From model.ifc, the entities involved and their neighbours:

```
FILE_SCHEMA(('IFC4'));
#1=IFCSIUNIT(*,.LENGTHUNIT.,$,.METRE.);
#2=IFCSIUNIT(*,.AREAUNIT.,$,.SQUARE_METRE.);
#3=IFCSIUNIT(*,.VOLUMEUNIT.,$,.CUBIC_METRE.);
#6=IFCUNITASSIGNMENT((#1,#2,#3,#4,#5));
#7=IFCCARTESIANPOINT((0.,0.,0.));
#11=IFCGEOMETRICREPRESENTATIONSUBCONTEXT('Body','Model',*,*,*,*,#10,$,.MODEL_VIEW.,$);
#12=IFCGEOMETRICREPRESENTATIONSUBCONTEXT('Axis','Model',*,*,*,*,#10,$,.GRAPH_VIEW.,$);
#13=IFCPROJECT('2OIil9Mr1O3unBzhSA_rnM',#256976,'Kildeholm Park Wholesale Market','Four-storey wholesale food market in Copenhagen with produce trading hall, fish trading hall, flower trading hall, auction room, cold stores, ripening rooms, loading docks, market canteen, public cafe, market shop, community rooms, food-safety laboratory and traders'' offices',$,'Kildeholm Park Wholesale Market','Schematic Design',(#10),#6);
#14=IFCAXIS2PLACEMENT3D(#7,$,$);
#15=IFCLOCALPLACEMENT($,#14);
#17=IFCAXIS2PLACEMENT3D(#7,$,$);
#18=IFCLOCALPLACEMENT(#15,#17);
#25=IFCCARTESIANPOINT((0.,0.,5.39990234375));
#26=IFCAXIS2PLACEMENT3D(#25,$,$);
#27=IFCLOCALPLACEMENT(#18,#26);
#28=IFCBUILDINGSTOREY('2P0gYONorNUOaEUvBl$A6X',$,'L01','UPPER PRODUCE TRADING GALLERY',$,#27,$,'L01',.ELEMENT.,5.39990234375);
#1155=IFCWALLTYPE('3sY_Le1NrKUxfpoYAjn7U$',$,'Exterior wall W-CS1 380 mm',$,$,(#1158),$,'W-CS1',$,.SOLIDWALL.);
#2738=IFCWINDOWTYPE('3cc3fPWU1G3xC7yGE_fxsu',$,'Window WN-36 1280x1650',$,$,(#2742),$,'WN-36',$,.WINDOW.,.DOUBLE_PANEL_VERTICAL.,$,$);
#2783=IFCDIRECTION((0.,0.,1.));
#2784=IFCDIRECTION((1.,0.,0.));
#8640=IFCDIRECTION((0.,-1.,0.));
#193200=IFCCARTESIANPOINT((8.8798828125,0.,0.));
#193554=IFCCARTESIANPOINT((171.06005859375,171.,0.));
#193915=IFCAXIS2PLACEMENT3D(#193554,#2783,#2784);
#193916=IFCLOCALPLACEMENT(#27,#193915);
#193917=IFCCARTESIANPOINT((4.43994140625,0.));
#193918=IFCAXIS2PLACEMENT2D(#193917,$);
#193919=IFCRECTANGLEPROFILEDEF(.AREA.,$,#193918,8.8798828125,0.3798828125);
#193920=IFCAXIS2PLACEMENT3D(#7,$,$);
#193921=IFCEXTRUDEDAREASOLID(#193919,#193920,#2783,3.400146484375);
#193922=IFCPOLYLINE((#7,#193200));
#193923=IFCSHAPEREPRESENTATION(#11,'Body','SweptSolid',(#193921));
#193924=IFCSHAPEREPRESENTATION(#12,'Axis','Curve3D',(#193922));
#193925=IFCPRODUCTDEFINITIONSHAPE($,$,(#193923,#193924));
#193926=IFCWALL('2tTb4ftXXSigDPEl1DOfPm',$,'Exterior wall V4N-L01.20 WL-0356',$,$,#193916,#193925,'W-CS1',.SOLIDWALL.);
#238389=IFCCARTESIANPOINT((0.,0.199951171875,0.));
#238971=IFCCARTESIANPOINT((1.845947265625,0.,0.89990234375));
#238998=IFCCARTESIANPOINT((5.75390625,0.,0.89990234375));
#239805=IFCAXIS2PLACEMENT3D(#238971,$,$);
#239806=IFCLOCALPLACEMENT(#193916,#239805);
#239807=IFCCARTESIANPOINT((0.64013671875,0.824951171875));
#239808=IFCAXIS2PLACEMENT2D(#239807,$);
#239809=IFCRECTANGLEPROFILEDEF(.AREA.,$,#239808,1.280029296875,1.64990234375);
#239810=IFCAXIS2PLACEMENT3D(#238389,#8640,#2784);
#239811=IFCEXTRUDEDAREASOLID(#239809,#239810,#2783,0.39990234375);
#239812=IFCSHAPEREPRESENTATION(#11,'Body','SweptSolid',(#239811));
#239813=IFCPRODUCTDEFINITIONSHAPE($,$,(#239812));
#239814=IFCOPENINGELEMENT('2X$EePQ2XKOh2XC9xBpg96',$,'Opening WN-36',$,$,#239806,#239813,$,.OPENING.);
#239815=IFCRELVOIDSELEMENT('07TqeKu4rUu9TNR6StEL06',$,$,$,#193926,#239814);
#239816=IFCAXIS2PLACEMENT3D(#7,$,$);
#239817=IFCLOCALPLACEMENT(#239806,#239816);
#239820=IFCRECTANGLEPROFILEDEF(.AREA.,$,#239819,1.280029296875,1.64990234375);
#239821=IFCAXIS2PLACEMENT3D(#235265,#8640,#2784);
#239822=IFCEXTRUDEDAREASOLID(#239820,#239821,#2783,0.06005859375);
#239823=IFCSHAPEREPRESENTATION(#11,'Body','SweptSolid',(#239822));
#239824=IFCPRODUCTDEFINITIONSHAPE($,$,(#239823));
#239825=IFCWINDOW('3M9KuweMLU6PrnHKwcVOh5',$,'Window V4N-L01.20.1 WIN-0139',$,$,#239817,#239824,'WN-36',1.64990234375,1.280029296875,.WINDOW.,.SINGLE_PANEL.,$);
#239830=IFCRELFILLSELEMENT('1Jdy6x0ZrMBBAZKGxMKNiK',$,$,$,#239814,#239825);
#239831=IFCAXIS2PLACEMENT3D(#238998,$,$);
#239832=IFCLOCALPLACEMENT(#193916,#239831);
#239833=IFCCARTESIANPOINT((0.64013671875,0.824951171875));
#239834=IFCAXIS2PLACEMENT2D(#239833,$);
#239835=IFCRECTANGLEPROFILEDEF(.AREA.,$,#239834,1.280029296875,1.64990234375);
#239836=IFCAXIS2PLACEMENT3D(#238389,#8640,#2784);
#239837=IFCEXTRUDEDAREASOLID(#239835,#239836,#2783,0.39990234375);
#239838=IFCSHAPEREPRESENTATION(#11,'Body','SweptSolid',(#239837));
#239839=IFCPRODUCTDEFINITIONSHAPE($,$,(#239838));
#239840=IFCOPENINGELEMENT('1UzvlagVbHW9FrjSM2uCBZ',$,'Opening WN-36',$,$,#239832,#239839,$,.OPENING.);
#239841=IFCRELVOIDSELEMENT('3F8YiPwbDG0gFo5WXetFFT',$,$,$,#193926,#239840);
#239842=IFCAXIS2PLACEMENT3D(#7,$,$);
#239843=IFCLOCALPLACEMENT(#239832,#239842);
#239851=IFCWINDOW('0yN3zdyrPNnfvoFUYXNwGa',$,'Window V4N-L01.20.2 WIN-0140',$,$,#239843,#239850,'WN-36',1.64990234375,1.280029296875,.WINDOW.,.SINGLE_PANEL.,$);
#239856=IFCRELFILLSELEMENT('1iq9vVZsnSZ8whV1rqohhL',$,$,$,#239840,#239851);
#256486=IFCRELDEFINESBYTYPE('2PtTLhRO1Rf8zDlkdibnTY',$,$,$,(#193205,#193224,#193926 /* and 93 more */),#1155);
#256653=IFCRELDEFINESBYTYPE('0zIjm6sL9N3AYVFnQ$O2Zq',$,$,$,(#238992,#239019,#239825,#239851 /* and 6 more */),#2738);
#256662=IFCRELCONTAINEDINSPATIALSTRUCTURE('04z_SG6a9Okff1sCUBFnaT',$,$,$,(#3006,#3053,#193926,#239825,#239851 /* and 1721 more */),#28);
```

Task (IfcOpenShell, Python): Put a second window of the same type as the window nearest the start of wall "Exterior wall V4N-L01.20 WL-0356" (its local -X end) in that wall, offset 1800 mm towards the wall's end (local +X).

```python
import ifcopenshell
import ifcopenshell.api.feature
import ifcopenshell.api.geometry
import ifcopenshell.api.root
import ifcopenshell.geom
import ifcopenshell.util.element
import ifcopenshell.util.placement
import ifcopenshell.util.shape
import ifcopenshell.util.unit

model = ifcopenshell.open("model.ifc")
unit_scale = ifcopenshell.util.unit.calculate_unit_scale(model)
settings = ifcopenshell.geom.settings()


def volume(element):
    """Net volume in cubic metres, openings subtracted."""
    shape = ifcopenshell.geom.create_shape(settings, element)
    return ifcopenshell.util.shape.get_volume(shape.geometry)


window = model.by_id(239825)
opening = window.FillsVoids[0].RelatingOpeningElement
wall = opening.VoidsElements[0].RelatingBuildingElement
before = volume(wall)
shift = ifcopenshell.util.placement.get_local_placement(wall.ObjectPlacement)[:3, 0] * 1.8 / unit_scale

# copy_class copies the void relationship, type, container and properties, but no geometry.
new_opening = ifcopenshell.api.root.copy_class(model, product=opening)
new_opening.Representation = ifcopenshell.util.element.copy_deep(
    model, opening.Representation, exclude=["IfcGeometricRepresentationContext", "IfcRepresentationMap"]
)
new_window = ifcopenshell.api.root.copy_class(model, product=window)
new_window.Representation = ifcopenshell.util.element.copy_deep(
    model, window.Representation, exclude=["IfcGeometricRepresentationContext", "IfcRepresentationMap"]
)
new_window.Tag = None
ifcopenshell.api.feature.add_filling(model, opening=new_opening, element=new_window)

for old, new in ((opening, new_opening), (window, new_window)):
    matrix = ifcopenshell.util.placement.get_local_placement(old.ObjectPlacement)
    matrix[:3, 3] += shift
    ifcopenshell.api.geometry.edit_object_placement(model, product=new, matrix=matrix, is_si=False)

after = volume(wall)

print(f"wall volume {before:.3f} -> {after:.3f} m3")

model.write("model_edited.ifc")
```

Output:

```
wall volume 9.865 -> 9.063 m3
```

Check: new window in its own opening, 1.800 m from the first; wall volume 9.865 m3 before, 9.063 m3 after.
